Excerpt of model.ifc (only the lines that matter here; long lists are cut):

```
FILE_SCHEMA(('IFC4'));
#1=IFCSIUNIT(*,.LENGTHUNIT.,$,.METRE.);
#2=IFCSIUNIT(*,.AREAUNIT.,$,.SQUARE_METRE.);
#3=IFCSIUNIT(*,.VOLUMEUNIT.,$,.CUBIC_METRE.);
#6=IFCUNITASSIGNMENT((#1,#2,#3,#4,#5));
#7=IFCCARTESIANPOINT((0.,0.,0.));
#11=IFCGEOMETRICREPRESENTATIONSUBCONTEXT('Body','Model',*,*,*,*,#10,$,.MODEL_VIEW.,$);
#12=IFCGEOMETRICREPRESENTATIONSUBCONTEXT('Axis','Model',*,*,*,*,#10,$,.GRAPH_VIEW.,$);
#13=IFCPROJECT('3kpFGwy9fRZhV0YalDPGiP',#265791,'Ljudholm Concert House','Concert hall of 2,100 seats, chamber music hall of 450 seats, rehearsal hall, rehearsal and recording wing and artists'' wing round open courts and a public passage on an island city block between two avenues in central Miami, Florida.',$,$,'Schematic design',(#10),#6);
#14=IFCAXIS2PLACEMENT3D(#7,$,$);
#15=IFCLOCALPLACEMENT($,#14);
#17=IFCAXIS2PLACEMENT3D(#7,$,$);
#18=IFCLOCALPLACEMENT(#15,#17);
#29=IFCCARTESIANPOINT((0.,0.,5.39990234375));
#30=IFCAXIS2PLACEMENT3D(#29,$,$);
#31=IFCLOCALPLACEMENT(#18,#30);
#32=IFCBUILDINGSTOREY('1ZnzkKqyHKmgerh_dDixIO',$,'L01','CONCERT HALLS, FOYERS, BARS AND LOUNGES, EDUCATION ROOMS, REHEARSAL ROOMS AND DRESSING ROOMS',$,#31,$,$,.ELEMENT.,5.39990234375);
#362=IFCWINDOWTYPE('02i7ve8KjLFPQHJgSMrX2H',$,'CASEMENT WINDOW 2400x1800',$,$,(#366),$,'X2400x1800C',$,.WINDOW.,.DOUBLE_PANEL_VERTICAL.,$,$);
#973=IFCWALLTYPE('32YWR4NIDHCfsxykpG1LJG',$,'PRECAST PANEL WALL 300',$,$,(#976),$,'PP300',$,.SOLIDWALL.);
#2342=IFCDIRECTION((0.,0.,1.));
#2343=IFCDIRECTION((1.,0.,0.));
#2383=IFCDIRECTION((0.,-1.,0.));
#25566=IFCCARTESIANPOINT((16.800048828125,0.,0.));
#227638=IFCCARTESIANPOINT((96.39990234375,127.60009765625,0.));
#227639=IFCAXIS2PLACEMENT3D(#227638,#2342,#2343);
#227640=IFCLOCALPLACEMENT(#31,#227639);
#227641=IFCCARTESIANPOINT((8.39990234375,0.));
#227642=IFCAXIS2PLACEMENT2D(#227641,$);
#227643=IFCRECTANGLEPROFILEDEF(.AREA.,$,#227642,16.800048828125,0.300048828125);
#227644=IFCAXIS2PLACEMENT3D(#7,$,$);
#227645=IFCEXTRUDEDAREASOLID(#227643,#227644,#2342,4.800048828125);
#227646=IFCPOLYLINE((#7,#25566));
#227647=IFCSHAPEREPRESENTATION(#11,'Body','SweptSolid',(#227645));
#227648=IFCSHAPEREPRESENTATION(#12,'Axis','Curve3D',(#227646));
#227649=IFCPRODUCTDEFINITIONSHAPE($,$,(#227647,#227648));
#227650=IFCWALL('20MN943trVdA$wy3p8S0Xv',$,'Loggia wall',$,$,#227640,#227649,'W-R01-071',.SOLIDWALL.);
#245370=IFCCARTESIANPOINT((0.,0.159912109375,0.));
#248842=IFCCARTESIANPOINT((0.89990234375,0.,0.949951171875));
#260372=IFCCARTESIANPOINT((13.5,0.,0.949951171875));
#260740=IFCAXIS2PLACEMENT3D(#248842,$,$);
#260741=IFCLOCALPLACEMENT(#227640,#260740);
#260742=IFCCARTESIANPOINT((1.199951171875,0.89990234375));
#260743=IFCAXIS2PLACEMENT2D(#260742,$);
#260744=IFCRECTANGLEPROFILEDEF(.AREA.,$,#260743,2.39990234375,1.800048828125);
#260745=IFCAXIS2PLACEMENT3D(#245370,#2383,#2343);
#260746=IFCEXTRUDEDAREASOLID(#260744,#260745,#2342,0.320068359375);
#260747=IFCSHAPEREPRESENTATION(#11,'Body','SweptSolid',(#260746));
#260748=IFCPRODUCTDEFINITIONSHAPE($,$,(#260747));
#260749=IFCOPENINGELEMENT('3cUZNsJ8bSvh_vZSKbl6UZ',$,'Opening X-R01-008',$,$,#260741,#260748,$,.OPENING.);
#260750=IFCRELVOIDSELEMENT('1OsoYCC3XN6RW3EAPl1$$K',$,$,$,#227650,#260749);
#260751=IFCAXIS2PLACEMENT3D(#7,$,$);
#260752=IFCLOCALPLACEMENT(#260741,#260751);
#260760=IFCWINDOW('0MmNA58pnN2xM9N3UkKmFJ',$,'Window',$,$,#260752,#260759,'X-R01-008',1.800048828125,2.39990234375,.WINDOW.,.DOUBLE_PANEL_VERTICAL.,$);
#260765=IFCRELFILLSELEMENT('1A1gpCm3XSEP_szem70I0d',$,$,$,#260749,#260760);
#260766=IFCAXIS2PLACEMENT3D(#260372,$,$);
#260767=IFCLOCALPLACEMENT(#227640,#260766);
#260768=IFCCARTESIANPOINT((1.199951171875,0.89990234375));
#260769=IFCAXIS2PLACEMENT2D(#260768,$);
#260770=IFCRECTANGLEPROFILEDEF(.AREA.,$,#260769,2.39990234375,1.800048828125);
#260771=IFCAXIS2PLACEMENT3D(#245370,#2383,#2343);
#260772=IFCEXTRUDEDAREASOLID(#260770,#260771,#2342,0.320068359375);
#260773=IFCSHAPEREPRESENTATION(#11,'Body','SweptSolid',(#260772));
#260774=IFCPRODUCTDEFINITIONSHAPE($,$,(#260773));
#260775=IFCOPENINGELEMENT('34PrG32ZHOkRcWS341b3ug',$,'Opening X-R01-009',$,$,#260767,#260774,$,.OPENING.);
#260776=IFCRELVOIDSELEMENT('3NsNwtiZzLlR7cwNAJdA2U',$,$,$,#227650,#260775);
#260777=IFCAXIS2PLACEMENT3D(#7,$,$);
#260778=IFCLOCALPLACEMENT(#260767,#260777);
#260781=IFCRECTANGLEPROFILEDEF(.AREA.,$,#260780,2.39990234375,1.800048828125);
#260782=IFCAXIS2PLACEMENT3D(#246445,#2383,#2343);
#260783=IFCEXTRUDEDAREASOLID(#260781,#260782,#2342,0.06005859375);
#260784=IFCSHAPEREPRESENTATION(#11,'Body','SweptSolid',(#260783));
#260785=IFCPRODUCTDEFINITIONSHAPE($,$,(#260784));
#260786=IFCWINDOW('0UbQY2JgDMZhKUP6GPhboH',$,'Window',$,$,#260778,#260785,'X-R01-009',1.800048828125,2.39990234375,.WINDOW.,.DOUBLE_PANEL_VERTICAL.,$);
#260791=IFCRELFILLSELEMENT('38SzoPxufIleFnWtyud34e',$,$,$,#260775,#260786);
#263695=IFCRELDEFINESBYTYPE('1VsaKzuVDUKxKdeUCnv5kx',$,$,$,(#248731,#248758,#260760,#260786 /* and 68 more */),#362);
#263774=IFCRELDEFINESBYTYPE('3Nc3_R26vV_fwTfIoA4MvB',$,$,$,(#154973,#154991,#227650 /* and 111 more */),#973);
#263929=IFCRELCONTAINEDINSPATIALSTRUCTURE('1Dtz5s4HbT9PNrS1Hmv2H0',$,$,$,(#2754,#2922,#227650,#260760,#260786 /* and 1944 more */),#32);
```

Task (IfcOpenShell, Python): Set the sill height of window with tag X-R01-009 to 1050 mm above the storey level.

```python
import numpy as np
import ifcopenshell
import ifcopenshell.api.geometry
import ifcopenshell.geom
import ifcopenshell.util.element
import ifcopenshell.util.placement
import ifcopenshell.util.shape
import ifcopenshell.util.unit

model = ifcopenshell.open("model.ifc")
unit_scale = ifcopenshell.util.unit.calculate_unit_scale(model)

window = model.by_id(260786)
opening = window.FillsVoids[0].RelatingOpeningElement
storey = ifcopenshell.util.element.get_container(window, ifc_class="IfcBuildingStorey")
level = ifcopenshell.util.placement.get_local_placement(storey.ObjectPlacement)[2, 3]

# The opening's origin need not be at the sill, so measure its lowest point.
shape = ifcopenshell.geom.create_shape(ifcopenshell.geom.settings(), opening)
bottom = ifcopenshell.util.shape.get_shape_bottom_elevation(shape, shape.geometry) / unit_scale
dz = level + 1.05 - bottom

shift = np.array([0.0, 0.0, dz])
# The window is placed relative to its opening, so it follows when the opening moves.
matrix = ifcopenshell.util.placement.get_local_placement(opening.ObjectPlacement)
matrix[:3, 3] += shift
ifcopenshell.api.geometry.edit_object_placement(
    model, product=opening, matrix=matrix, is_si=False, should_transform_children=True
)

print(f"moved by {dz * unit_scale:+.3f} m")

model.write("model-out.ifc")
```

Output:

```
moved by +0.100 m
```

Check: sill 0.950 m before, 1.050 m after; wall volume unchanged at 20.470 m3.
